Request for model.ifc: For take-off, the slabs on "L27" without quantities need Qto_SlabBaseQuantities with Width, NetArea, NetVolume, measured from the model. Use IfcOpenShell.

First a look at what the model holds.

```python
import ifcopenshell
import ifcopenshell.util.element
import ifcopenshell.util.unit

model = ifcopenshell.open("model.ifc")
print(model.schema)
for unit_type in ("LENGTHUNIT", "AREAUNIT", "VOLUMEUNIT"):
    print(unit_type, ifcopenshell.util.unit.calculate_unit_scale(model, unit_type))
storey = next(s for s in model.by_type("IfcBuildingStorey") if s.Name == "L27")
slabs = [e for e in ifcopenshell.util.element.get_decomposition(storey) if e.is_a("IfcSlab")]
for e in sorted(slabs, key=lambda e: e.id()):
    print(e.id(), e.is_a(), e.Name, list(ifcopenshell.util.element.get_psets(e, qtos_only=True)), sep=" | ")
```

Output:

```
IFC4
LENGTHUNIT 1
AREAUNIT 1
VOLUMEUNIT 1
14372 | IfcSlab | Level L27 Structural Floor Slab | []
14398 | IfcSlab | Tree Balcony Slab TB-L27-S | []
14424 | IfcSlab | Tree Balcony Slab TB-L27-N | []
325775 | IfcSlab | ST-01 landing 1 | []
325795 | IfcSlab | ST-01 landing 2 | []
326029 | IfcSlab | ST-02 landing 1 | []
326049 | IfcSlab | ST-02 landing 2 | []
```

```python
import ifcopenshell
import ifcopenshell.api.pset
import ifcopenshell.geom
import ifcopenshell.util.element
import ifcopenshell.util.shape
import ifcopenshell.util.unit

model = ifcopenshell.open("model.ifc")
unit_scale = ifcopenshell.util.unit.calculate_unit_scale(model)
area_scale = ifcopenshell.util.unit.calculate_unit_scale(model, "AREAUNIT")
volume_scale = ifcopenshell.util.unit.calculate_unit_scale(model, "VOLUMEUNIT")
settings = ifcopenshell.geom.settings()

storey = next(s for s in model.by_type("IfcBuildingStorey") if s.Name == "L27")
slabs = [e for e in ifcopenshell.util.element.get_decomposition(storey) if e.is_a("IfcSlab")]

for e in sorted(slabs, key=lambda e: e.id()):
    if ifcopenshell.util.element.get_psets(e, qtos_only=True, should_inherit=False):
        continue
    # Geometry comes back in metres, in the element's own axes.
    shape = ifcopenshell.geom.create_shape(settings, e)
    values = {
        "Width": ifcopenshell.util.shape.get_z(shape.geometry) / unit_scale,
        "NetArea": ifcopenshell.util.shape.get_footprint_area(shape.geometry) / area_scale,
        "NetVolume": ifcopenshell.util.shape.get_volume(shape.geometry) / volume_scale,
    }
    qto = ifcopenshell.api.pset.add_qto(model, product=e, name="Qto_SlabBaseQuantities")
    ifcopenshell.api.pset.edit_qto(model, qto=qto, properties=values)
    print(e.id(), {k: round(v, 3) for k, v in values.items()})

model.write("model_v2.ifc")
```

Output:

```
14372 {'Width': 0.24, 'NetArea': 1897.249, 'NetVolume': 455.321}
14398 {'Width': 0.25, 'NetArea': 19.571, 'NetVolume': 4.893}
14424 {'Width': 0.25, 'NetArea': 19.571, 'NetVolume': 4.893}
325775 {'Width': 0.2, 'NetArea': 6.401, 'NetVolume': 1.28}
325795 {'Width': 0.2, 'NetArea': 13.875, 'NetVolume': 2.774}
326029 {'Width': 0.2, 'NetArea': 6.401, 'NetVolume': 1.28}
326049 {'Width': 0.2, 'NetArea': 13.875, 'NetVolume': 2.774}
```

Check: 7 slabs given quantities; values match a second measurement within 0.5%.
